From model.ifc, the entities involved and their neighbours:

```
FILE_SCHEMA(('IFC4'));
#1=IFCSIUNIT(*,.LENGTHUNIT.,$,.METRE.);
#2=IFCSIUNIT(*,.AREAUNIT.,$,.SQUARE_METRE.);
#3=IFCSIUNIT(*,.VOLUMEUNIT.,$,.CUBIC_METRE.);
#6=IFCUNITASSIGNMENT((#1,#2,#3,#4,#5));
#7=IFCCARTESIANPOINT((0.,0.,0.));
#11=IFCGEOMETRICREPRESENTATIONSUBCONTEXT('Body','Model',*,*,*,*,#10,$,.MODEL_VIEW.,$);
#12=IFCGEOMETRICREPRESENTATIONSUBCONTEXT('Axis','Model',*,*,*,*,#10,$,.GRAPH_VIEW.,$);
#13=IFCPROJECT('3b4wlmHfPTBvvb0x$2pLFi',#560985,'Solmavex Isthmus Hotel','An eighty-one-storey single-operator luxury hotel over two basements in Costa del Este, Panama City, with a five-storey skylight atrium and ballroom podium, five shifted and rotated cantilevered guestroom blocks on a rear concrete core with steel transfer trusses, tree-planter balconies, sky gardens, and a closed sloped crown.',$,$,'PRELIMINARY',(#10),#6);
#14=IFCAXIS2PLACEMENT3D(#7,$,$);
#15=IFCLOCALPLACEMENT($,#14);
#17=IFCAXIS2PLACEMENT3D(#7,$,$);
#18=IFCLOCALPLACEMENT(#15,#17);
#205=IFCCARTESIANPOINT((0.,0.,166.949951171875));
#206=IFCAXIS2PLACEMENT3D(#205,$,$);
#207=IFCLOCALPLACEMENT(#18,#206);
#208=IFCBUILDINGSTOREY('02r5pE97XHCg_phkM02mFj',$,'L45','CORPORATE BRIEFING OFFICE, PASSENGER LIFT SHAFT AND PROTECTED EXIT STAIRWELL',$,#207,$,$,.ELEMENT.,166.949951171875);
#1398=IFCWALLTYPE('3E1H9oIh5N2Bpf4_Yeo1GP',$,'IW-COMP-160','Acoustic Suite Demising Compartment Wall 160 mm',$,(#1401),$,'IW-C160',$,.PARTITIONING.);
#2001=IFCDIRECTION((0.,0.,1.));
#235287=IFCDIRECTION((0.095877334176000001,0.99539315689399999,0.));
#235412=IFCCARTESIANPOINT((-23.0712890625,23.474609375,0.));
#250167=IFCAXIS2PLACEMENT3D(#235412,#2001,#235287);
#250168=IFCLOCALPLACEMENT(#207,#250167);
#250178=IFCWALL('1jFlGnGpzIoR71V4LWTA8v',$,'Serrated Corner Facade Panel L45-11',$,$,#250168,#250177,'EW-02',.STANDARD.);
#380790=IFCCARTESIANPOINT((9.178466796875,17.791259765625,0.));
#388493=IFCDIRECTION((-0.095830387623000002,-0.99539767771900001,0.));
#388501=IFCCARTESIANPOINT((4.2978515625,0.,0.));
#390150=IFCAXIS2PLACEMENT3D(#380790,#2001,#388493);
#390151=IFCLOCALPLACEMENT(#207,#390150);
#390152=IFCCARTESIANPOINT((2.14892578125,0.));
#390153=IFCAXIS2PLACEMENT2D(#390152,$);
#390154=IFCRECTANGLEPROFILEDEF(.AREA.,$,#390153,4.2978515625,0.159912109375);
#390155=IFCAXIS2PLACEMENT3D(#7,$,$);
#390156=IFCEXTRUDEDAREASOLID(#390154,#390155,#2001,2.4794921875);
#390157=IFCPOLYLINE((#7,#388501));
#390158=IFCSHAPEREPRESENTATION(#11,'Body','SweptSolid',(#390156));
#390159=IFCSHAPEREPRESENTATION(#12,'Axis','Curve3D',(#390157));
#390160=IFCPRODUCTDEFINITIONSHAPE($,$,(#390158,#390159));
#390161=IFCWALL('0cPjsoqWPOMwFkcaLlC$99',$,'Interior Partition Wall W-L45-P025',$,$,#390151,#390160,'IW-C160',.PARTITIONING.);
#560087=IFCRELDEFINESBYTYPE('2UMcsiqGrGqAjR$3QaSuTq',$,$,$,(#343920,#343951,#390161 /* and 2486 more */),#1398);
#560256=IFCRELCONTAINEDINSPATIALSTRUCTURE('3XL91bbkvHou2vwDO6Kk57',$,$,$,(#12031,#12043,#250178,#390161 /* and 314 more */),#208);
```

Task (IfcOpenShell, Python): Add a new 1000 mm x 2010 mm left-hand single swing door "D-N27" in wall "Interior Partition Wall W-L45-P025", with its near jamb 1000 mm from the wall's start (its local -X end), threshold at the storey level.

```python
import numpy as np
import ifcopenshell
import ifcopenshell.api.feature
import ifcopenshell.api.geometry
import ifcopenshell.api.root
import ifcopenshell.api.spatial
import ifcopenshell.geom
import ifcopenshell.util.element
import ifcopenshell.util.placement
import ifcopenshell.util.representation
import ifcopenshell.util.shape
import ifcopenshell.util.unit

model = ifcopenshell.open("model.ifc")
unit_scale = ifcopenshell.util.unit.calculate_unit_scale(model)
settings = ifcopenshell.geom.settings()


def volume(element):
    """Net volume in cubic metres, openings subtracted."""
    shape = ifcopenshell.geom.create_shape(settings, element)
    return ifcopenshell.util.shape.get_volume(shape.geometry)


wall = model.by_guid("0cPjsoqWPOMwFkcaLlC$99")
storey = ifcopenshell.util.element.get_container(wall, ifc_class="IfcBuildingStorey")
context = ifcopenshell.util.representation.get_context(model, "Model", "Body", "MODEL_VIEW")
before = volume(wall)

width, height, from_end, sill = 1, 2.01, 1, 0.0  # metres

# The wall runs along its own X axis, and the end named is its -X end.
wall_shape = ifcopenshell.geom.create_shape(settings, wall)
x, y, z = ifcopenshell.util.shape.get_vertices(wall_shape.geometry).T
start = x.min() + from_end
face, thickness = float(y.min()), float(y.max() - y.min())
wall_matrix = ifcopenshell.util.placement.get_local_placement(wall.ObjectPlacement)
level = ifcopenshell.util.placement.get_local_placement(storey.ObjectPlacement)[2, 3]


def in_wall(x, y):
    """Placement at x, y metres in the wall's axes, at sill height."""
    matrix = wall_matrix.copy()
    matrix[:, 3] = wall_matrix @ np.array([x / unit_scale, y / unit_scale, 0.0, 1.0])
    matrix[2, 3] = level + sill / unit_scale
    return matrix


# Opening: a box that overshoots both wall faces by 50 mm.
opening = ifcopenshell.api.root.create_entity(model, ifc_class="IfcOpeningElement", predefined_type="OPENING")
box = ifcopenshell.api.geometry.add_wall_representation(
    model, context=context, length=width, height=height, thickness=thickness + 0.1
)
ifcopenshell.api.geometry.assign_representation(model, product=opening, representation=box)
ifcopenshell.api.geometry.edit_object_placement(model, product=opening, matrix=in_wall(start, face - 0.05), is_si=False)
ifcopenshell.api.feature.add_feature(model, feature=opening, element=wall)

door = ifcopenshell.api.root.create_entity(model, ifc_class="IfcDoor", name="D-N27", predefined_type="DOOR")
door.OverallWidth, door.OverallHeight = width / unit_scale, height / unit_scale
door.OperationType = "SINGLE_SWING_LEFT"
body = ifcopenshell.api.geometry.add_door_representation(
    model,
    context=context,
    overall_width=door.OverallWidth,
    overall_height=door.OverallHeight,
    operation_type="SINGLE_SWING_LEFT",
    lining_properties={"LiningDepth": thickness / unit_scale, "ThresholdDepth": thickness / unit_scale},
)
ifcopenshell.api.geometry.assign_representation(model, product=door, representation=body)
ifcopenshell.api.spatial.assign_container(model, products=[door], relating_structure=storey)
ifcopenshell.api.feature.add_filling(model, opening=opening, element=door)

# The lining spans the wall, so the door starts at the wall face.
ifcopenshell.api.geometry.edit_object_placement(model, product=door, matrix=in_wall(start, face), is_si=False)

after = volume(wall)

print(f"wall volume {before:.3f} -> {after:.3f} m3")

model.write("model_rev.ifc")
```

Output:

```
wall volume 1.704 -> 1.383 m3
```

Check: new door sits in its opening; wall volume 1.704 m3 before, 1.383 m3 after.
